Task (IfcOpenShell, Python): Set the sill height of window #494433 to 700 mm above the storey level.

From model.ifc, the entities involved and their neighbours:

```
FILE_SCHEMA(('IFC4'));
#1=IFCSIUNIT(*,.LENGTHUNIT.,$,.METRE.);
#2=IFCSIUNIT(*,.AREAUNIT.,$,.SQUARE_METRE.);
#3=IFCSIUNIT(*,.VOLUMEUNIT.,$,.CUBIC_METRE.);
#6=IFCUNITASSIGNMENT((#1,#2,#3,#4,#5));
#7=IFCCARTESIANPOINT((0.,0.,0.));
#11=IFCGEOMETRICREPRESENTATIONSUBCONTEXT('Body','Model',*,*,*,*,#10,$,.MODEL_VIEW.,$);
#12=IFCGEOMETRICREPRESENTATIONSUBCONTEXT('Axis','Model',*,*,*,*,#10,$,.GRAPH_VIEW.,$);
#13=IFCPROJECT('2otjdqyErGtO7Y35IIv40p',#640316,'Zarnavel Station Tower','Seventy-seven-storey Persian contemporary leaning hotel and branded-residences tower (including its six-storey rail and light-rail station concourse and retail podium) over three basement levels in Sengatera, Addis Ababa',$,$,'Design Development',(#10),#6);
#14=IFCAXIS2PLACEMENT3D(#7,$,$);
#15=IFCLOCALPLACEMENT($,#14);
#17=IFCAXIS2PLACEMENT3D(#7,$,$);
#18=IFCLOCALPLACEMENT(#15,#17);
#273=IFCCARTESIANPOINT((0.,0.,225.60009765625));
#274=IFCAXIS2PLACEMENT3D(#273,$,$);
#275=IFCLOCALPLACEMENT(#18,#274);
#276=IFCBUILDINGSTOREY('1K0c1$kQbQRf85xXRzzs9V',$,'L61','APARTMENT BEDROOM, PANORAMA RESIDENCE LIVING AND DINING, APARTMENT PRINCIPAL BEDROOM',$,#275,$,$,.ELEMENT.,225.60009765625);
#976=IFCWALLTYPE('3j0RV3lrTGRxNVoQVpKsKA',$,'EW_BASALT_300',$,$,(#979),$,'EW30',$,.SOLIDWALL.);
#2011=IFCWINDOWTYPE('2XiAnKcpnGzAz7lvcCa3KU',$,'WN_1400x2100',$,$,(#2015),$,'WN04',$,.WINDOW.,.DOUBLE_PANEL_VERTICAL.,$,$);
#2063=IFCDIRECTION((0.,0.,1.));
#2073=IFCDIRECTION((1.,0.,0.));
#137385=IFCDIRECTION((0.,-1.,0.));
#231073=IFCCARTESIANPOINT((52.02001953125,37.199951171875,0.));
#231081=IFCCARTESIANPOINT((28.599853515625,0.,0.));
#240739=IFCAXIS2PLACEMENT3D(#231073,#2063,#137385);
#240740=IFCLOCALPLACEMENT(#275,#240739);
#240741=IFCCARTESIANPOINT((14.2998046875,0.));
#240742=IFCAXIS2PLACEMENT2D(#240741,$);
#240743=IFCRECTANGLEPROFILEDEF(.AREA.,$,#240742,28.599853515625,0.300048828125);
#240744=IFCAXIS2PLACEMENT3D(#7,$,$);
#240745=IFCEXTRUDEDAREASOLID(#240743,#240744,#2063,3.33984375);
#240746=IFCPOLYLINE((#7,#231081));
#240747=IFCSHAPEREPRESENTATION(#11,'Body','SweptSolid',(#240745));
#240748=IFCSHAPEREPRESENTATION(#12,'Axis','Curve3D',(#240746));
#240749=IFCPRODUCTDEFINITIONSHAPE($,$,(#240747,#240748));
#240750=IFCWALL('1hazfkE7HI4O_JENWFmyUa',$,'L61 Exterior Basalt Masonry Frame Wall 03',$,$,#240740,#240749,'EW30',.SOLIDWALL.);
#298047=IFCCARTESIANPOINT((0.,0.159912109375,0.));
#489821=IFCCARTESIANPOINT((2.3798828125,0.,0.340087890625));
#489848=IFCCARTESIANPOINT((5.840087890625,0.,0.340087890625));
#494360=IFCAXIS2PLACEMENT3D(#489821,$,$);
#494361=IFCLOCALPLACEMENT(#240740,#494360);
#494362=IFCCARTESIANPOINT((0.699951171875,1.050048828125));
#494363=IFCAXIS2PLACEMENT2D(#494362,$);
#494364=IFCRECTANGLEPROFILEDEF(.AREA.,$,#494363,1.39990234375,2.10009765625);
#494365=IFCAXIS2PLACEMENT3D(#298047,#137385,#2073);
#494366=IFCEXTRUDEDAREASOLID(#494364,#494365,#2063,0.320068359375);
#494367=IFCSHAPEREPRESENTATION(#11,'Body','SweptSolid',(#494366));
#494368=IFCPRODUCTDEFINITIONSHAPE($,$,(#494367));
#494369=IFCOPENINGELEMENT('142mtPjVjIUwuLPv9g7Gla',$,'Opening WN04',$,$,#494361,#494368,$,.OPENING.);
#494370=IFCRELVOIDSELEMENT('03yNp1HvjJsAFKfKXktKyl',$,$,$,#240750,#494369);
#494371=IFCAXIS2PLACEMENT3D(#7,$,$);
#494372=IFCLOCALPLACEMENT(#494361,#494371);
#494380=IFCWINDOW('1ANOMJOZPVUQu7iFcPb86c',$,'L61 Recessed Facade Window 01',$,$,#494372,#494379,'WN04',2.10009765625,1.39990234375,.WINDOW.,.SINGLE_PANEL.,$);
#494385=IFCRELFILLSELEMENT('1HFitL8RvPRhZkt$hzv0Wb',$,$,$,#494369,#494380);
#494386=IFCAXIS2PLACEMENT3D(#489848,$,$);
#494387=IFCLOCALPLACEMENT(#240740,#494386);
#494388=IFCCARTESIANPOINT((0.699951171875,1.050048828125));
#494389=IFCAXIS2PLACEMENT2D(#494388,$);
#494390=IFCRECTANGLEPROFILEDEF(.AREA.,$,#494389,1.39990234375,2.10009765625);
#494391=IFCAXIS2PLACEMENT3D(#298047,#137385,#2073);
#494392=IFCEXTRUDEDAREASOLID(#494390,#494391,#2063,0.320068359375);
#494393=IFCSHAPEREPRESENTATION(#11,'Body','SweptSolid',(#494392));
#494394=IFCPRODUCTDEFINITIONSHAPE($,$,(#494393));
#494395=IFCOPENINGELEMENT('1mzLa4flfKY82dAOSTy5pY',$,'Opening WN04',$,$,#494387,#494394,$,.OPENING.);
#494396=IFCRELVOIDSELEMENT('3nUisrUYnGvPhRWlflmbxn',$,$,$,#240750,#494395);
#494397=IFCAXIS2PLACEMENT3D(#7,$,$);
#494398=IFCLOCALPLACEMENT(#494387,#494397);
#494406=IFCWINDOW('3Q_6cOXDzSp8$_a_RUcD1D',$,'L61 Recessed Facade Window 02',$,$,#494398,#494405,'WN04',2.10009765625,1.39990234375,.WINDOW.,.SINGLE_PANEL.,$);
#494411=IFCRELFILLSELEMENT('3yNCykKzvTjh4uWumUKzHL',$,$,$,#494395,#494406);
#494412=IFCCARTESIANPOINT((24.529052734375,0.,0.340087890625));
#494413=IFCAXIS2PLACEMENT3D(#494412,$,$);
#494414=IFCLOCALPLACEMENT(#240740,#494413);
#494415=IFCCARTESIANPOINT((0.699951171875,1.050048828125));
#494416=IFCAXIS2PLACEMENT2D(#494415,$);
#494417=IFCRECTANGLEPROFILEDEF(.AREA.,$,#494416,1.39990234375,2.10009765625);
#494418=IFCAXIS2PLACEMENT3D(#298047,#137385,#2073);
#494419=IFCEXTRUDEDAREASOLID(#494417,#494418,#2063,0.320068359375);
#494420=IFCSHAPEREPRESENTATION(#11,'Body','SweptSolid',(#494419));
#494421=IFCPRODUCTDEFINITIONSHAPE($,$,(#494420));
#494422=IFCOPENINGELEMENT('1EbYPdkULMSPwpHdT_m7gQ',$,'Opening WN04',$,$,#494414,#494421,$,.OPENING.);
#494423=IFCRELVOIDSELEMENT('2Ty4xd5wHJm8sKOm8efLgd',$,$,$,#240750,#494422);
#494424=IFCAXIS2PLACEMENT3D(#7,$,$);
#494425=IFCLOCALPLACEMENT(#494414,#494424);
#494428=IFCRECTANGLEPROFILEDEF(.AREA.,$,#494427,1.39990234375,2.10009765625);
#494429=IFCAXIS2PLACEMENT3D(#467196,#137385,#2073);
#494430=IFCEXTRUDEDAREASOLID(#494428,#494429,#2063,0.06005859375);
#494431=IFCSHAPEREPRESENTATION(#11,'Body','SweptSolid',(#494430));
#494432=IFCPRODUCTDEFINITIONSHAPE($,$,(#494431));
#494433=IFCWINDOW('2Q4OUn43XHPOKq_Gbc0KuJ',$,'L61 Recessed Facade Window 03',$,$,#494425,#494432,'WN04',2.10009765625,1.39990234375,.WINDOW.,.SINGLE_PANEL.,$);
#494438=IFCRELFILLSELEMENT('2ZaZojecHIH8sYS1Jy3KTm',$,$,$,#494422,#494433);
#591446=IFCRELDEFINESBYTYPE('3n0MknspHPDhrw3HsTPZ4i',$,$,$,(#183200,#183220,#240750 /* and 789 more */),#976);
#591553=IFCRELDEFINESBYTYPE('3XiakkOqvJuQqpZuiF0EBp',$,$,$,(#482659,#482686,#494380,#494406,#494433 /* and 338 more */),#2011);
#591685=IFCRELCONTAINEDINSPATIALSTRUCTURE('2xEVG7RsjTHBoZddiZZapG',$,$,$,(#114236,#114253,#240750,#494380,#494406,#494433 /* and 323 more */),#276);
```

```python
import numpy as np
import ifcopenshell
import ifcopenshell.api.geometry
import ifcopenshell.geom
import ifcopenshell.util.element
import ifcopenshell.util.placement
import ifcopenshell.util.shape
import ifcopenshell.util.unit

model = ifcopenshell.open("model.ifc")
unit_scale = ifcopenshell.util.unit.calculate_unit_scale(model)

window = model.by_id(494433)
opening = window.FillsVoids[0].RelatingOpeningElement
storey = ifcopenshell.util.element.get_container(window, ifc_class="IfcBuildingStorey")
level = ifcopenshell.util.placement.get_local_placement(storey.ObjectPlacement)[2, 3]

# The opening's origin need not be at the sill, so measure its lowest point.
shape = ifcopenshell.geom.create_shape(ifcopenshell.geom.settings(), opening)
bottom = ifcopenshell.util.shape.get_shape_bottom_elevation(shape, shape.geometry) / unit_scale
dz = level + 0.7 - bottom

shift = np.array([0.0, 0.0, dz])
# The window is placed relative to its opening, so it follows when the opening moves.
matrix = ifcopenshell.util.placement.get_local_placement(opening.ObjectPlacement)
matrix[:3, 3] += shift
ifcopenshell.api.geometry.edit_object_placement(
    model, product=opening, matrix=matrix, is_si=False, should_transform_children=True
)

print(f"moved by {dz * unit_scale:+.3f} m")

model.write("model-out.ifc")
```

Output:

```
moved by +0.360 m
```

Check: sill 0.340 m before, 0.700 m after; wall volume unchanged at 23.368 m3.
